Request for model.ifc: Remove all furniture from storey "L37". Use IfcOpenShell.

First a look at what the model holds.

```python
import ifcopenshell
import ifcopenshell.util.element

model = ifcopenshell.open("model.ifc")
print(model.schema)
storey = next(s for s in model.by_type("IfcBuildingStorey") if s.Name == "L37")
furniture = [e for e in ifcopenshell.util.element.get_decomposition(storey) if e.is_a("IfcFurnishingElement")]
seen = {}
for e in furniture:
    element_type = ifcopenshell.util.element.get_type(e)
    name = element_type.Name if element_type not in (None, e) else None
    seen[name] = seen.get(name, 0) + 1
for name, count in sorted(seen.items(), key=str):
    print(count, "x", name)
```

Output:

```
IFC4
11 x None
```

```python
import ifcopenshell
import ifcopenshell.api.root
import ifcopenshell.util.element

model = ifcopenshell.open("model.ifc")

storey = next(s for s in model.by_type("IfcBuildingStorey") if s.Name == "L37")
furniture = [e for e in ifcopenshell.util.element.get_decomposition(storey) if e.is_a("IfcFurnishingElement")]

for e in furniture:
    ifcopenshell.api.root.remove_product(model, product=e)
print(len(furniture), "removed")

model.write("model_updated.ifc")
```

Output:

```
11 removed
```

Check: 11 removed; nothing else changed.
